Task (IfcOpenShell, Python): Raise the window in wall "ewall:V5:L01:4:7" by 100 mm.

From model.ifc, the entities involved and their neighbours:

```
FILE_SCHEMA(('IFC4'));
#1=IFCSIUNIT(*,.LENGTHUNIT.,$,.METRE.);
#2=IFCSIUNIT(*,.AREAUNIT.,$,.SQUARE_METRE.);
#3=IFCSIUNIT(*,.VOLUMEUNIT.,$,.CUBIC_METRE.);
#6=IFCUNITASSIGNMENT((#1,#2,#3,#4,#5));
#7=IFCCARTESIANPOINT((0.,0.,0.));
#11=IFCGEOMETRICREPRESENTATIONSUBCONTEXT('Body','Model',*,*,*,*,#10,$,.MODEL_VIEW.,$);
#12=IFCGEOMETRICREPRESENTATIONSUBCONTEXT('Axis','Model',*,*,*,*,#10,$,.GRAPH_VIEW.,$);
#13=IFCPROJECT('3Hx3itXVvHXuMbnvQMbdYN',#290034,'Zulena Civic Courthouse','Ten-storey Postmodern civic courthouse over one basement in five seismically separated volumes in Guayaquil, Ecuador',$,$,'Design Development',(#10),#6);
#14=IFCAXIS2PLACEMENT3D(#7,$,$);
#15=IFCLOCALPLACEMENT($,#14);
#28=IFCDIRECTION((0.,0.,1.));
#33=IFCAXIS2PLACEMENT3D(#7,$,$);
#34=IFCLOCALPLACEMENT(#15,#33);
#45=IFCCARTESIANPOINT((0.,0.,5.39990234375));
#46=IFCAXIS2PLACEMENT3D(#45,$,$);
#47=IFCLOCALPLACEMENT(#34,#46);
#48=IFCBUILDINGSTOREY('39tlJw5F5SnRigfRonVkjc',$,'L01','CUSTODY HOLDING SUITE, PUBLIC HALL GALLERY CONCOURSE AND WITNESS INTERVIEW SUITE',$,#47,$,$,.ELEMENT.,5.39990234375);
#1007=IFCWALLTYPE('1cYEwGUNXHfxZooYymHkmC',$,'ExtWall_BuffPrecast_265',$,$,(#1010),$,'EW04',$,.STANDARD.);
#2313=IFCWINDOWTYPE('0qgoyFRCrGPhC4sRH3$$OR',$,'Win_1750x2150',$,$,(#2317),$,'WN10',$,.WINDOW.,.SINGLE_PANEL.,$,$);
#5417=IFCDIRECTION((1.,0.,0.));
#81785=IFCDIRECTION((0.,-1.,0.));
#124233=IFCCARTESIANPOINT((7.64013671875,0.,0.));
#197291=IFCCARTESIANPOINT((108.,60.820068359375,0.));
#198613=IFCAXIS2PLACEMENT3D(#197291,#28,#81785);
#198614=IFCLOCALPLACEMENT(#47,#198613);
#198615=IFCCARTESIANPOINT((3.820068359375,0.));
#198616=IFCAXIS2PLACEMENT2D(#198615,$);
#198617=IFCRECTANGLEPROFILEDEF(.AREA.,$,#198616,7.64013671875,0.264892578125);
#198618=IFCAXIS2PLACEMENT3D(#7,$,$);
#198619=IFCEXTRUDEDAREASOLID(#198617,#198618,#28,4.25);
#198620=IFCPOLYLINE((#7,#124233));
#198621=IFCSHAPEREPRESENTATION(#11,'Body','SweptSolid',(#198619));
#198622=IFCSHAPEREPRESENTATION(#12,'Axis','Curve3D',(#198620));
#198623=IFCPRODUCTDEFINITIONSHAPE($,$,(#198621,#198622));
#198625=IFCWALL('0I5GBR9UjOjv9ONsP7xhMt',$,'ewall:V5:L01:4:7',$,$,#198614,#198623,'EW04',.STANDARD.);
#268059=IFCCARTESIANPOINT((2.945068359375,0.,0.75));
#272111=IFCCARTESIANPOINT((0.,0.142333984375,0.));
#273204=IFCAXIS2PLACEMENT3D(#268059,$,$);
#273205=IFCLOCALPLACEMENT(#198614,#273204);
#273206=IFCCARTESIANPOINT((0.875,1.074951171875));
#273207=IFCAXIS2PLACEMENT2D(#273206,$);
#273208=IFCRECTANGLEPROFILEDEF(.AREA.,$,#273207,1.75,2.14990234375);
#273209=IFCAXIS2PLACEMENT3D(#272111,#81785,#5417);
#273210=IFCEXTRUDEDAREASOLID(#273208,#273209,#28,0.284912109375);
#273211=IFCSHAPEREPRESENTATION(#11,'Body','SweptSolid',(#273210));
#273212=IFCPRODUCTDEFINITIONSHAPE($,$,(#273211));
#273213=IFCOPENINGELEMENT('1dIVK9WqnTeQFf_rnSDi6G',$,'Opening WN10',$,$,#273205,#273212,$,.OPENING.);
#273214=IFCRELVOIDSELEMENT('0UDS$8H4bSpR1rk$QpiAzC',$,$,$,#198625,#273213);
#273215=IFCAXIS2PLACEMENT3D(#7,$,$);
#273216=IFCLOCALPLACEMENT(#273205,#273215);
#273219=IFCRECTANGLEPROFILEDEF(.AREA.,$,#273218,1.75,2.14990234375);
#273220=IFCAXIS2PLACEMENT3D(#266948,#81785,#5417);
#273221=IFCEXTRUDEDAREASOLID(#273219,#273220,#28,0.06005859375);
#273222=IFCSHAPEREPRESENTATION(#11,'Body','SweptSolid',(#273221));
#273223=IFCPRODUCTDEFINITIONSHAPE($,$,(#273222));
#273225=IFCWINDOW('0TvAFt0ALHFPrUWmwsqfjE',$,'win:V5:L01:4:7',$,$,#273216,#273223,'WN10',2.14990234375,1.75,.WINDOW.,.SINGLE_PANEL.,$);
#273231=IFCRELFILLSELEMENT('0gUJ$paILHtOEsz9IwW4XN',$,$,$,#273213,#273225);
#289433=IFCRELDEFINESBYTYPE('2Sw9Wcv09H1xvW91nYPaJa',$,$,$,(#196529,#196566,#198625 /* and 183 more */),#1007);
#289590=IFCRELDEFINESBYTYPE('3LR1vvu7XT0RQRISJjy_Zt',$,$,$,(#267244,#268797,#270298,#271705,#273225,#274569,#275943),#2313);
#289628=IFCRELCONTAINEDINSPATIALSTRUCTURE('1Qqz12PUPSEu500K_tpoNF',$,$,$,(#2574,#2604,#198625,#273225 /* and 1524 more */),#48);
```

```python
import numpy as np
import ifcopenshell
import ifcopenshell.api.geometry
import ifcopenshell.util.placement
import ifcopenshell.util.unit

model = ifcopenshell.open("model.ifc")
unit_scale = ifcopenshell.util.unit.calculate_unit_scale(model)

window = model.by_id(273225)
opening = window.FillsVoids[0].RelatingOpeningElement
dz = 0.1 / unit_scale

shift = np.array([0.0, 0.0, dz])
# The window is placed relative to its opening, so it follows when the opening moves.
matrix = ifcopenshell.util.placement.get_local_placement(opening.ObjectPlacement)
matrix[:3, 3] += shift
ifcopenshell.api.geometry.edit_object_placement(
    model, product=opening, matrix=matrix, is_si=False, should_transform_children=True
)

print(f"moved by {dz * unit_scale:+.3f} m")

model.write("model_v2.ifc")
```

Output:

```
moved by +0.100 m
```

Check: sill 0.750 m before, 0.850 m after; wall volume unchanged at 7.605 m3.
